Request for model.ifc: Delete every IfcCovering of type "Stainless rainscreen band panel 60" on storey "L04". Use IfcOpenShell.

First a look at what the model holds.

```python
import ifcopenshell
import ifcopenshell.util.element

model = ifcopenshell.open("model.ifc")
print(model.schema)
storey = next(s for s in model.by_type("IfcBuildingStorey") if s.Name == "L04")
coverings = [e for e in ifcopenshell.util.element.get_decomposition(storey) if e.is_a("IfcCovering")]
seen = {}
for e in coverings:
    element_type = ifcopenshell.util.element.get_type(e)
    name = element_type.Name if element_type not in (None, e) else None
    seen[name] = seen.get(name, 0) + 1
for name, count in sorted(seen.items(), key=str):
    print(count, "x", name)
```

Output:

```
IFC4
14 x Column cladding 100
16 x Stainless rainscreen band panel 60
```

```python
import ifcopenshell
import ifcopenshell.api.root
import ifcopenshell.util.element

model = ifcopenshell.open("model.ifc")

storey = next(s for s in model.by_type("IfcBuildingStorey") if s.Name == "L04")
coverings = [e for e in ifcopenshell.util.element.get_decomposition(storey) if e.is_a("IfcCovering")]
targets = [e for e in coverings if (t := ifcopenshell.util.element.get_type(e)) not in (None, e) and t.Name == "Stainless rainscreen band panel 60"]

for e in targets:
    ifcopenshell.api.root.remove_product(model, product=e)
print(len(targets), "removed")

model.write("model_edited.ifc")
```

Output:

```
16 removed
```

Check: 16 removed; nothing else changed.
